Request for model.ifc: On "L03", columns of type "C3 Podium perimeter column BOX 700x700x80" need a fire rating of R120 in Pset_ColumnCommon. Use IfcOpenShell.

First a look at what the model holds.

```python
import ifcopenshell
import ifcopenshell.util.element

model = ifcopenshell.open("model.ifc")
print(model.schema)
storey = next(s for s in model.by_type("IfcBuildingStorey") if s.Name == "L03")
columns = [e for e in ifcopenshell.util.element.get_decomposition(storey) if e.is_a("IfcColumn")]
seen = {}
for e in columns:
    element_type = ifcopenshell.util.element.get_type(e)
    key = (element_type.Name if element_type != e and element_type else None, ifcopenshell.util.element.get_pset(e, "Pset_ColumnCommon", "FireRating"))
    seen[key] = seen.get(key, 0) + 1
for (name, value), count in sorted(seen.items(), key=str):
    print(count, "x", name, "|", value)
```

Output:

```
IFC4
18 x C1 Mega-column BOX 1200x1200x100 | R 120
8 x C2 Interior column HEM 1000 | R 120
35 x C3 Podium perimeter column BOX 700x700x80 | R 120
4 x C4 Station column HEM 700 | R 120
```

```python
import ifcopenshell
import ifcopenshell.api.pset
import ifcopenshell.util.element

model = ifcopenshell.open("model.ifc")

storey = next(s for s in model.by_type("IfcBuildingStorey") if s.Name == "L03")
columns = [e for e in ifcopenshell.util.element.get_decomposition(storey) if e.is_a("IfcColumn")]

count = 0
for e in columns:
    element_type = ifcopenshell.util.element.get_type(e)
    if element_type in (None, e) or element_type.Name != "C3 Podium perimeter column BOX 700x700x80":
        continue
    found = ifcopenshell.util.element.get_pset(e, "Pset_ColumnCommon", should_inherit=False)
    if found:
        pset = model.by_id(found["id"])
        if len(ifcopenshell.util.element.get_elements_by_pset(pset)) > 1:
            pset = ifcopenshell.api.pset.unshare_pset(model, products=[e], pset=pset)[0]
    else:
        pset = ifcopenshell.api.pset.add_pset(model, product=e, name="Pset_ColumnCommon")
    ifcopenshell.api.pset.edit_pset(model, pset=pset, properties={"FireRating": "R120"})
    count += 1

print(count, "columns updated")

model.write("model_v2.ifc")
```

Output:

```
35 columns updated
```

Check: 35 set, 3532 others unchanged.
